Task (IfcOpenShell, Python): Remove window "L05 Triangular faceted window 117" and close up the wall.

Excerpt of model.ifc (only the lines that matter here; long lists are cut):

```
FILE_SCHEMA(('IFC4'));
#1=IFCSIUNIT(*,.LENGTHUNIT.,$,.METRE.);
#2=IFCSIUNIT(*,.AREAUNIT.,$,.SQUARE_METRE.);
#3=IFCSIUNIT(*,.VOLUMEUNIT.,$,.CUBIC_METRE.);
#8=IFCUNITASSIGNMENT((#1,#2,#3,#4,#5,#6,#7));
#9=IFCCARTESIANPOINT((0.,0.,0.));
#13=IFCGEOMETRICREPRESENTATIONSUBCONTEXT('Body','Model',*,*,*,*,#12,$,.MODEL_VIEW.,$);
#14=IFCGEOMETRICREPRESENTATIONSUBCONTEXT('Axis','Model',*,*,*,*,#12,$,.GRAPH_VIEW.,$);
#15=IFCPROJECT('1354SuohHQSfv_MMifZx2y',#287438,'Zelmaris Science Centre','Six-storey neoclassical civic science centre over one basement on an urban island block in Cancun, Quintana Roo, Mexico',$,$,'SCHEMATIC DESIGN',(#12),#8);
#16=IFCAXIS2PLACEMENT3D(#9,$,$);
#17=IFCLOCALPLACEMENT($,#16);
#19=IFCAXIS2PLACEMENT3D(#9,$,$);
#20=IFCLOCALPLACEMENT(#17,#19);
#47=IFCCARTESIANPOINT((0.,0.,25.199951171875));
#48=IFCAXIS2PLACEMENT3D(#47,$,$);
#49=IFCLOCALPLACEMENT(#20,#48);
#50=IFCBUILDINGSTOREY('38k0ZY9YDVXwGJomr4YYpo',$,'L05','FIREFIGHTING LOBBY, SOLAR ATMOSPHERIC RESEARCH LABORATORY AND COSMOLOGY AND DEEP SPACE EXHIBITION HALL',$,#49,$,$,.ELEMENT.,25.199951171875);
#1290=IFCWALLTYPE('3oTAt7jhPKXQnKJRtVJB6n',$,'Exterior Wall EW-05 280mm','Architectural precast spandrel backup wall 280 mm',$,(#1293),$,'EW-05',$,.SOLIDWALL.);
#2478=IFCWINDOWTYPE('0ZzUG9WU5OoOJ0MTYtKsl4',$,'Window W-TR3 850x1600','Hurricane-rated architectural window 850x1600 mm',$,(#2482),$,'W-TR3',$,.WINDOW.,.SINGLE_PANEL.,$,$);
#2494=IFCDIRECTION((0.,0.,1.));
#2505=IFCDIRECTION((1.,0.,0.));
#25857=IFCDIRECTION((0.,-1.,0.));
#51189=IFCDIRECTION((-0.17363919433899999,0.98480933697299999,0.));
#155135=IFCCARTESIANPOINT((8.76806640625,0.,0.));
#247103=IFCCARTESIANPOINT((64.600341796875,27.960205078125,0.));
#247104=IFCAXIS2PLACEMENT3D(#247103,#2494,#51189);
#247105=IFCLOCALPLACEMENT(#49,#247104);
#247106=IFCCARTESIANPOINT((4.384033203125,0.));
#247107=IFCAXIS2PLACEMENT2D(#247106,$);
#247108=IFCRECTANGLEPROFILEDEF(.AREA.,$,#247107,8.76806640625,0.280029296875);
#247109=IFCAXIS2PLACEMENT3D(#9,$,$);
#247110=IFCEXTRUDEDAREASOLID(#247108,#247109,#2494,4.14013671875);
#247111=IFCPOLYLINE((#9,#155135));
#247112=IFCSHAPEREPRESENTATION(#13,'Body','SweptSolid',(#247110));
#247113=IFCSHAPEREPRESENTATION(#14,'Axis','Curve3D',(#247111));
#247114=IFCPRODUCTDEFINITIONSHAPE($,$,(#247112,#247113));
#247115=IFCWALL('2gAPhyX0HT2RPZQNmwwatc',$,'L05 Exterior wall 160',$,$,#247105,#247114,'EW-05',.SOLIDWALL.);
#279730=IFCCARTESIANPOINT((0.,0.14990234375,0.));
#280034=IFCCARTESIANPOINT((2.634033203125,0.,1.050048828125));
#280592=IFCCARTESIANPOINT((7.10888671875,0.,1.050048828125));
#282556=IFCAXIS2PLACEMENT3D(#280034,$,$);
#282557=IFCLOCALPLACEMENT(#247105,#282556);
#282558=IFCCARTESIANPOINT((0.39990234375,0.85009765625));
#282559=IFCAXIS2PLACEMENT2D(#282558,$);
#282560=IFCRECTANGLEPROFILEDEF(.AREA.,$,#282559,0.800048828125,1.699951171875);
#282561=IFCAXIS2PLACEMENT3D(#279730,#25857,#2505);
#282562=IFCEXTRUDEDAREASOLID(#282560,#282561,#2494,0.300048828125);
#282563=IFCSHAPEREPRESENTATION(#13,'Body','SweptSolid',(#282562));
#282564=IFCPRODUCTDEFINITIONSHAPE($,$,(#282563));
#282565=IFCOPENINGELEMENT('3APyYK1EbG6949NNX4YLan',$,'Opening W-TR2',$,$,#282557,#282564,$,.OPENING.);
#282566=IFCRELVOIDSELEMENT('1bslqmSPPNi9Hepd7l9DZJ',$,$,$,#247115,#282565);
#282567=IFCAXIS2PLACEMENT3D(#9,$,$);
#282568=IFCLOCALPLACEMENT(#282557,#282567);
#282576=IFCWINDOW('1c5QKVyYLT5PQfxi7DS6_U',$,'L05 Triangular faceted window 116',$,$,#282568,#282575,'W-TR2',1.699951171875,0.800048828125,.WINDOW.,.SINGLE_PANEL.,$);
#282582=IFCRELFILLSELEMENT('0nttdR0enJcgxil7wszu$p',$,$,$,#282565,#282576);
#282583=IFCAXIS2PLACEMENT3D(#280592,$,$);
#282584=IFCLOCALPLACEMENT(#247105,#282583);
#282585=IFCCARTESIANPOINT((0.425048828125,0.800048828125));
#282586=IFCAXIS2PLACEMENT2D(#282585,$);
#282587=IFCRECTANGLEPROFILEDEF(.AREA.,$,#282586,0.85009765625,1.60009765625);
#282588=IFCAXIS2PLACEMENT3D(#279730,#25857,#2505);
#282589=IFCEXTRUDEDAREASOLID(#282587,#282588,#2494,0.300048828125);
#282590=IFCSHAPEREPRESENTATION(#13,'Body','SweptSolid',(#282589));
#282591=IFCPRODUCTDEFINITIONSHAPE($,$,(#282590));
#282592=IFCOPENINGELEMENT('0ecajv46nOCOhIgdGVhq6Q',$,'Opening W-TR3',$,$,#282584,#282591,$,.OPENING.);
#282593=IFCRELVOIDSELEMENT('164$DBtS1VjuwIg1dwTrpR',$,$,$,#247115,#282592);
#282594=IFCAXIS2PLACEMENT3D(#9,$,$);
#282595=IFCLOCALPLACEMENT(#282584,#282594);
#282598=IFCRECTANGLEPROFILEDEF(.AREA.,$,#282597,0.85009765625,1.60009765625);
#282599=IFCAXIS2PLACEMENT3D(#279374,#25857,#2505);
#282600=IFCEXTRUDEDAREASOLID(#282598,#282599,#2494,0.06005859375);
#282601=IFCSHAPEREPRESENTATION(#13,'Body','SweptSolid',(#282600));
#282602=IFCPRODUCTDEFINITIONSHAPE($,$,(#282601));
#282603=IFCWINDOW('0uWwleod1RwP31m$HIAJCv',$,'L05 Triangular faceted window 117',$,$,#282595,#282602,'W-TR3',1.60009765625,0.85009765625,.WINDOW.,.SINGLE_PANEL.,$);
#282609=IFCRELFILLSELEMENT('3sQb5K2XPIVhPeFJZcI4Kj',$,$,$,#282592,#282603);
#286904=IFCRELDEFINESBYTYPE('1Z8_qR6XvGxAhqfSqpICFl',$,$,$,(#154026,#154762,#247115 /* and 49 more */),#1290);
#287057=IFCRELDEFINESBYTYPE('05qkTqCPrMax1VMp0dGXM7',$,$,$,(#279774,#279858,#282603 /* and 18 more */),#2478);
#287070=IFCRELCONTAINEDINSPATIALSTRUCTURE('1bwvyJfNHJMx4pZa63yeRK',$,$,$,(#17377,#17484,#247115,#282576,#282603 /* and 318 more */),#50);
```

```python
import ifcopenshell
import ifcopenshell.api.feature
import ifcopenshell.api.root
import ifcopenshell.geom
import ifcopenshell.util.shape

model = ifcopenshell.open("model.ifc")
settings = ifcopenshell.geom.settings()


def volume(element):
    """Net volume in cubic metres, openings subtracted."""
    shape = ifcopenshell.geom.create_shape(settings, element)
    return ifcopenshell.util.shape.get_volume(shape.geometry)


window = model.by_guid("0uWwleod1RwP31m$HIAJCv")
opening = window.FillsVoids[0].RelatingOpeningElement
wall = opening.VoidsElements[0].RelatingBuildingElement
before = volume(wall)

ifcopenshell.api.root.remove_product(model, product=window)
ifcopenshell.api.feature.remove_feature(model, feature=opening)

after = volume(wall)

print(f"wall volume {before:.3f} -> {after:.3f} m3")

model.write("model_updated.ifc")
```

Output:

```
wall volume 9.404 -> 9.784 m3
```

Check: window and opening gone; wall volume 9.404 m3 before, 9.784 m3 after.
